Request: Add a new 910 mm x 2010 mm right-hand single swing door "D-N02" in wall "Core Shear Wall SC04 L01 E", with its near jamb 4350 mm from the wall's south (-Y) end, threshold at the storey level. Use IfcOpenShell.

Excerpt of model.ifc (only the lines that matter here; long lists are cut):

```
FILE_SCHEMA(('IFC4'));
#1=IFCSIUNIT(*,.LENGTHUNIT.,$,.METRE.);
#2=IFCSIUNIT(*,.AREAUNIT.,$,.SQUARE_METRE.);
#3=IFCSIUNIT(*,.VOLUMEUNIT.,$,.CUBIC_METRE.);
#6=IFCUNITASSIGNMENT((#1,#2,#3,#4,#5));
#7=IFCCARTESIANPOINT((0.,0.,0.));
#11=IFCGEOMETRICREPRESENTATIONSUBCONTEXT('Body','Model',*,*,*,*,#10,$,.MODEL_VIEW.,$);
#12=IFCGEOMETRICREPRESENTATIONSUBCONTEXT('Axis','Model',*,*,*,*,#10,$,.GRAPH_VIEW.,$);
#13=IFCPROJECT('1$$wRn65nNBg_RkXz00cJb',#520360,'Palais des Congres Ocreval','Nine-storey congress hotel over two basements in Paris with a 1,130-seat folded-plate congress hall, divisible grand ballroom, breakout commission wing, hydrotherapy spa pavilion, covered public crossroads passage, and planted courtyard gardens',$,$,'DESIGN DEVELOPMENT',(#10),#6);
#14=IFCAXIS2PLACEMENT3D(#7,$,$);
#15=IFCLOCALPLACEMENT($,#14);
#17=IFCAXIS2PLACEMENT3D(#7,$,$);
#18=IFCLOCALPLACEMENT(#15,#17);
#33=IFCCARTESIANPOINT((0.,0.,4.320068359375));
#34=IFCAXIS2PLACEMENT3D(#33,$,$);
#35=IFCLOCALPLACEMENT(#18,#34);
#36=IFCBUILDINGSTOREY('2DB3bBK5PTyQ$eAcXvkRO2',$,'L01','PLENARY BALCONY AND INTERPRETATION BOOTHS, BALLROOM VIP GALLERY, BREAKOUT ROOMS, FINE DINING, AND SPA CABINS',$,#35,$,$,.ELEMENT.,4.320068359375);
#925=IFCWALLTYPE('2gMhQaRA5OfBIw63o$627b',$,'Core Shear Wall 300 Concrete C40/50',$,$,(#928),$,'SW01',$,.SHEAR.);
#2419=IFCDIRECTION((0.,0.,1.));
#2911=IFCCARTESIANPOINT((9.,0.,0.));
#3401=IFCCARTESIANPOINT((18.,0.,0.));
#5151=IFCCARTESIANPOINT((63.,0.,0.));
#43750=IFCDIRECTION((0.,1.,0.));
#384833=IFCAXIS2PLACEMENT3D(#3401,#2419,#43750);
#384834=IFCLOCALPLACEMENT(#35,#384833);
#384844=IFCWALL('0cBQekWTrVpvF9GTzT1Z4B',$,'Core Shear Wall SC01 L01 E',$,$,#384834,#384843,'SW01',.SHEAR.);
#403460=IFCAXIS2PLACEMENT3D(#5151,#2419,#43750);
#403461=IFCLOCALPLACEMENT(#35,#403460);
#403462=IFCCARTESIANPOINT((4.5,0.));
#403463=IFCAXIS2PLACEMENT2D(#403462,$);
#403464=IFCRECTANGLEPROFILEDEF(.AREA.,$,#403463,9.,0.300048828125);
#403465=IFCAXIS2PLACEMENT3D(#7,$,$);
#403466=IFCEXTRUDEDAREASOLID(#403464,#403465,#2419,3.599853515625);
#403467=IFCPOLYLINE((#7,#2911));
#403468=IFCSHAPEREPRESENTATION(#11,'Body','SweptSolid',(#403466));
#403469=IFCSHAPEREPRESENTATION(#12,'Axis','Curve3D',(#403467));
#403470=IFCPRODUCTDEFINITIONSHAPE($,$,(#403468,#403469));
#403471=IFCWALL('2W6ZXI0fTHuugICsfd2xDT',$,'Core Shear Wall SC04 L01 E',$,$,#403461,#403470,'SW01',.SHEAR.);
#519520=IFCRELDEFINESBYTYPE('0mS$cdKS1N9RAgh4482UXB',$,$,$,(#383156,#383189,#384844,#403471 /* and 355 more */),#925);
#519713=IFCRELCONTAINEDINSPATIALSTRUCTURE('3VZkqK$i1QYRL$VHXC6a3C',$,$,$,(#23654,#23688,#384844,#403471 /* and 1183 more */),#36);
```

```python
import numpy as np
import ifcopenshell
import ifcopenshell.api.feature
import ifcopenshell.api.geometry
import ifcopenshell.api.root
import ifcopenshell.api.spatial
import ifcopenshell.geom
import ifcopenshell.util.element
import ifcopenshell.util.placement
import ifcopenshell.util.representation
import ifcopenshell.util.shape
import ifcopenshell.util.unit

model = ifcopenshell.open("model.ifc")
unit_scale = ifcopenshell.util.unit.calculate_unit_scale(model)
settings = ifcopenshell.geom.settings()


def volume(element):
    """Net volume in cubic metres, openings subtracted."""
    shape = ifcopenshell.geom.create_shape(settings, element)
    return ifcopenshell.util.shape.get_volume(shape.geometry)


wall = model.by_id(403471)
storey = ifcopenshell.util.element.get_container(wall, ifc_class="IfcBuildingStorey")
context = ifcopenshell.util.representation.get_context(model, "Model", "Body", "MODEL_VIEW")
before = volume(wall)

width, height, from_end, sill = 0.91, 2.01, 4.35, 0.0  # metres

# The wall runs along its own X axis, and the end named is its -X end.
wall_shape = ifcopenshell.geom.create_shape(settings, wall)
x, y, z = ifcopenshell.util.shape.get_vertices(wall_shape.geometry).T
start = x.min() + from_end
face, thickness = float(y.min()), float(y.max() - y.min())
wall_matrix = ifcopenshell.util.placement.get_local_placement(wall.ObjectPlacement)
level = ifcopenshell.util.placement.get_local_placement(storey.ObjectPlacement)[2, 3]


def in_wall(x, y):
    """Placement at x, y metres in the wall's axes, at sill height."""
    matrix = wall_matrix.copy()
    matrix[:, 3] = wall_matrix @ np.array([x / unit_scale, y / unit_scale, 0.0, 1.0])
    matrix[2, 3] = level + sill / unit_scale
    return matrix


# Opening: a box that overshoots both wall faces by 50 mm.
opening = ifcopenshell.api.root.create_entity(model, ifc_class="IfcOpeningElement", predefined_type="OPENING")
box = ifcopenshell.api.geometry.add_wall_representation(
    model, context=context, length=width, height=height, thickness=thickness + 0.1
)
ifcopenshell.api.geometry.assign_representation(model, product=opening, representation=box)
ifcopenshell.api.geometry.edit_object_placement(model, product=opening, matrix=in_wall(start, face - 0.05), is_si=False)
ifcopenshell.api.feature.add_feature(model, feature=opening, element=wall)

door = ifcopenshell.api.root.create_entity(model, ifc_class="IfcDoor", name="D-N02", predefined_type="DOOR")
door.OverallWidth, door.OverallHeight = width / unit_scale, height / unit_scale
door.OperationType = "SINGLE_SWING_RIGHT"
body = ifcopenshell.api.geometry.add_door_representation(
    model,
    context=context,
    overall_width=door.OverallWidth,
    overall_height=door.OverallHeight,
    operation_type="SINGLE_SWING_RIGHT",
    lining_properties={"LiningDepth": thickness / unit_scale, "ThresholdDepth": thickness / unit_scale},
)
ifcopenshell.api.geometry.assign_representation(model, product=door, representation=body)
ifcopenshell.api.spatial.assign_container(model, products=[door], relating_structure=storey)
ifcopenshell.api.feature.add_filling(model, opening=opening, element=door)

# The lining spans the wall, so the door starts at the wall face.
ifcopenshell.api.geometry.edit_object_placement(model, product=door, matrix=in_wall(start, face), is_si=False)

after = volume(wall)

print(f"wall volume {before:.3f} -> {after:.3f} m3")

model.write("model_v2.ifc")
```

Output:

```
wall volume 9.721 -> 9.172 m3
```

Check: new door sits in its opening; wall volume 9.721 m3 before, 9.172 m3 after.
